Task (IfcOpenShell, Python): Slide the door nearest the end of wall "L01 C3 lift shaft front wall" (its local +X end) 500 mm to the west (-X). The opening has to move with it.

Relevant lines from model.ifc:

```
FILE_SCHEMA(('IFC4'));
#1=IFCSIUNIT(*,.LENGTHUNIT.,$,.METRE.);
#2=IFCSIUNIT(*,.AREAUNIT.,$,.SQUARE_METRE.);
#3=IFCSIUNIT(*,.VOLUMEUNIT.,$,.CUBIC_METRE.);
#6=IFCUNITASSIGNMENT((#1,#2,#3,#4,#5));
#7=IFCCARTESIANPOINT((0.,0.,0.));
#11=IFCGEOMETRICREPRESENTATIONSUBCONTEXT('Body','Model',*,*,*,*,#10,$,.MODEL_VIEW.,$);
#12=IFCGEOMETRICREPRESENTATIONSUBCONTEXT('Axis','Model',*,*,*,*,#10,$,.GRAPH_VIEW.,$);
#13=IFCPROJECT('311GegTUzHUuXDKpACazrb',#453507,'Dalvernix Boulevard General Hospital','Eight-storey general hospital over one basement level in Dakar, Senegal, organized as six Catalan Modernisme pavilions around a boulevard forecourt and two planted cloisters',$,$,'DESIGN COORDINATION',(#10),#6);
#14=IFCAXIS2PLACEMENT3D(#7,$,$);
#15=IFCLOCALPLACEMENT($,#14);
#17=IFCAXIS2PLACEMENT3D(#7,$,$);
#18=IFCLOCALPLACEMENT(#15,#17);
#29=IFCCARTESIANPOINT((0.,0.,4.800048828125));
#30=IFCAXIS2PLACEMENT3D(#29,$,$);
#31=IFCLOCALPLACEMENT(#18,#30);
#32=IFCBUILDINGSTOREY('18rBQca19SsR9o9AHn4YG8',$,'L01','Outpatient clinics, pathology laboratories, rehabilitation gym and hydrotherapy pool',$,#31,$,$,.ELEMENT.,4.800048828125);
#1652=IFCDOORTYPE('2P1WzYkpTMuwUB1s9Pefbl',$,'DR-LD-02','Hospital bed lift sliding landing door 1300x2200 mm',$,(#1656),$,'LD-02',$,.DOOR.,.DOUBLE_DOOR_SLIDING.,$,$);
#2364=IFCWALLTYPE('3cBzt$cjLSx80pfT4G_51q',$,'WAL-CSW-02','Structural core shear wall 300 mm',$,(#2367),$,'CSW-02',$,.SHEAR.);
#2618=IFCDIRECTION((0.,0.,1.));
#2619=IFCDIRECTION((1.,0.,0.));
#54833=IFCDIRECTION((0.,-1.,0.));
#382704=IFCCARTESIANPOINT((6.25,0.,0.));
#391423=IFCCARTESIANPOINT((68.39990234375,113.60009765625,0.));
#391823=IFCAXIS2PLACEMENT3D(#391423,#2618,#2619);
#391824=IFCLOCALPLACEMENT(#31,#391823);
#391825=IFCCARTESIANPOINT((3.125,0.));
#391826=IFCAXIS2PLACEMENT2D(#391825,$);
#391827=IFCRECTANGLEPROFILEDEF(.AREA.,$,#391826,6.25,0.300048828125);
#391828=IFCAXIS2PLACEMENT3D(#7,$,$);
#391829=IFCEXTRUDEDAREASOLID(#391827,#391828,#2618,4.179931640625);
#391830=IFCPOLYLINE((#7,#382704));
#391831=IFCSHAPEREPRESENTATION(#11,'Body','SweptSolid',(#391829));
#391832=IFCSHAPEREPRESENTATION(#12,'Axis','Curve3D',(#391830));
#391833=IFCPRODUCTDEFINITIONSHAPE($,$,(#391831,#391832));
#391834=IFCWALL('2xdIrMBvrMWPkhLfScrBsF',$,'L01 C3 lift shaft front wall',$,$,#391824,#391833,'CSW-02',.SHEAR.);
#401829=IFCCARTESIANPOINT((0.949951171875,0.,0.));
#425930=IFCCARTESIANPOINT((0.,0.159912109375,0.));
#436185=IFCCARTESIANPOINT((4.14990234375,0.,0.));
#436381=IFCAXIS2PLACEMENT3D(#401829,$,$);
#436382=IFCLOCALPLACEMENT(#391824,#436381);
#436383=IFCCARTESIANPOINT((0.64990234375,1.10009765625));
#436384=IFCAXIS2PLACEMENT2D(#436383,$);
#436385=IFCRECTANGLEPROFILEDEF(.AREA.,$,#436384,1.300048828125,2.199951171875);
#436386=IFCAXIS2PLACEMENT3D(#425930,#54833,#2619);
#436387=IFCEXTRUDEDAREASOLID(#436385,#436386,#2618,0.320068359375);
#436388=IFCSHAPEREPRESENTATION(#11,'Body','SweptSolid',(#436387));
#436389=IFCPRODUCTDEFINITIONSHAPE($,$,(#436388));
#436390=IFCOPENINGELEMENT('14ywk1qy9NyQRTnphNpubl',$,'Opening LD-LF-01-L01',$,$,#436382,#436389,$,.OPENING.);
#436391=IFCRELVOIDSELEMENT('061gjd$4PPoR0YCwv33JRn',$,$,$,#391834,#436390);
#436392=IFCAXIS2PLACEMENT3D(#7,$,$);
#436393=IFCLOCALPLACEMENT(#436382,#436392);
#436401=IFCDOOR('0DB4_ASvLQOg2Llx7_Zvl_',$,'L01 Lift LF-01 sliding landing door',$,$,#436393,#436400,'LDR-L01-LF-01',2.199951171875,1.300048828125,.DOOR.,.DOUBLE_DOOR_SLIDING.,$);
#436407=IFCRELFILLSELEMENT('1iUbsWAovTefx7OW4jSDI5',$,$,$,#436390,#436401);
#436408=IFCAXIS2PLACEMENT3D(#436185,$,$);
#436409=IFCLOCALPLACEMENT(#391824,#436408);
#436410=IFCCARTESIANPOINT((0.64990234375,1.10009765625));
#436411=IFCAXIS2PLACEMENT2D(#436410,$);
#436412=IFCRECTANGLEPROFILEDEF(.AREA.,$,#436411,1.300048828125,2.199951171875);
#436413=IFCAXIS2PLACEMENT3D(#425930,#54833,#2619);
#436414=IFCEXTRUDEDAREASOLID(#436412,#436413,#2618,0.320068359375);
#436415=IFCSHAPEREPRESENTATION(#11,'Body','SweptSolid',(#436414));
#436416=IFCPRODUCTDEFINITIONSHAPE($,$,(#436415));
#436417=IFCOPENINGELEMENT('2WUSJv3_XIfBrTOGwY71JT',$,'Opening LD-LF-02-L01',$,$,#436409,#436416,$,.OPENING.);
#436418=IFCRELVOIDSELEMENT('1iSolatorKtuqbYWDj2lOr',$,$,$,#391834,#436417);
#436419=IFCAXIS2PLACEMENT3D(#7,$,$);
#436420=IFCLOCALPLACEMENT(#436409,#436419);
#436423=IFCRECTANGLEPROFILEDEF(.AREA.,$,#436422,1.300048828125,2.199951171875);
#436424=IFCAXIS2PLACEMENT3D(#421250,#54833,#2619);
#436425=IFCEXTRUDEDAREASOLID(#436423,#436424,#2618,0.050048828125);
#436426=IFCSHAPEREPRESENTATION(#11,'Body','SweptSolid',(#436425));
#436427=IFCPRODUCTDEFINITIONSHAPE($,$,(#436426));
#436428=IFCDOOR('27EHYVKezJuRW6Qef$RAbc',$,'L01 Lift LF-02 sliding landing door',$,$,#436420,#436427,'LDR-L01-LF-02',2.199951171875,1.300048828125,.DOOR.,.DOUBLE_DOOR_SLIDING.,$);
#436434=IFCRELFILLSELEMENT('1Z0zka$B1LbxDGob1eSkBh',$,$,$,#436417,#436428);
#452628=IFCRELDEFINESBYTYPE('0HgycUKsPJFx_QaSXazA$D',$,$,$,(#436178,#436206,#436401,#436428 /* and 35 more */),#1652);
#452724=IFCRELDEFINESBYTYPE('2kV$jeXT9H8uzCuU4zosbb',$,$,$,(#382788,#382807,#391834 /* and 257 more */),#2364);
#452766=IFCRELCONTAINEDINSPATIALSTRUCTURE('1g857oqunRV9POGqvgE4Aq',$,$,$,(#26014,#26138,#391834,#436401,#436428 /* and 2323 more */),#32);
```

```python
import ifcopenshell
import ifcopenshell.api.geometry
import ifcopenshell.util.placement
import ifcopenshell.util.unit

model = ifcopenshell.open("model.ifc")
unit_scale = ifcopenshell.util.unit.calculate_unit_scale(model)

door = model.by_guid("27EHYVKezJuRW6Qef$RAbc")
opening = door.FillsVoids[0].RelatingOpeningElement
wall = opening.VoidsElements[0].RelatingBuildingElement

wall_matrix = ifcopenshell.util.placement.get_local_placement(wall.ObjectPlacement)
shift = wall_matrix[:3, 0] * -0.5 / unit_scale
before = ifcopenshell.util.placement.get_local_placement(door.ObjectPlacement)[:3, 3].copy()

# The door is placed relative to its opening, so it follows when the opening moves.
matrix = ifcopenshell.util.placement.get_local_placement(opening.ObjectPlacement)
matrix[:3, 3] += shift
ifcopenshell.api.geometry.edit_object_placement(
    model, product=opening, matrix=matrix, is_si=False, should_transform_children=True
)

after = ifcopenshell.util.placement.get_local_placement(door.ObjectPlacement)[:3, 3]
print("door moved by", (after - before).round(3) + 0.0)

model.write("model_rev.ifc")
```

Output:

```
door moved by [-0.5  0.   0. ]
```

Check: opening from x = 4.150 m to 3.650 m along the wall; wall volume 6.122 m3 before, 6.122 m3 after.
